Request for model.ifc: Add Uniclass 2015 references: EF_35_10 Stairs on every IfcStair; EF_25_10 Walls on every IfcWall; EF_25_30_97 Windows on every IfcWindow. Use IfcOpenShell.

First a look at what the model holds.

```python
import ifcopenshell

model = ifcopenshell.open("model.ifc")
print(model.schema)
print("classifications:", [c.Name for c in model.by_type("IfcClassification")])
for ifc_class in ("IfcDoor", "IfcRoof", "IfcStair", "IfcWall", "IfcWindow"):
    print(ifc_class, len(model.by_type(ifc_class)))
```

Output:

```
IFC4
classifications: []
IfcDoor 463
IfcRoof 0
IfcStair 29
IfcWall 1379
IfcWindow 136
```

```python
import ifcopenshell
import ifcopenshell.api.classification

model = ifcopenshell.open("model.ifc")

system = ifcopenshell.api.classification.add_classification(model, classification="Uniclass 2015")

codes = {
    "IfcStair": ("EF_35_10", "Stairs"),
    "IfcWall": ("EF_25_10", "Walls"),
    "IfcWindow": ("EF_25_30_97", "Windows"),
}
for ifc_class, (code, name) in codes.items():
    products = model.by_type(ifc_class)
    ifcopenshell.api.classification.add_reference(
        model, products=products, classification=system, identification=code, name=name
    )
    print(code, len(products))

model.write("model-out.ifc")
```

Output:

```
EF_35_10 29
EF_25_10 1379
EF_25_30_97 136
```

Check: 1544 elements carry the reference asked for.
